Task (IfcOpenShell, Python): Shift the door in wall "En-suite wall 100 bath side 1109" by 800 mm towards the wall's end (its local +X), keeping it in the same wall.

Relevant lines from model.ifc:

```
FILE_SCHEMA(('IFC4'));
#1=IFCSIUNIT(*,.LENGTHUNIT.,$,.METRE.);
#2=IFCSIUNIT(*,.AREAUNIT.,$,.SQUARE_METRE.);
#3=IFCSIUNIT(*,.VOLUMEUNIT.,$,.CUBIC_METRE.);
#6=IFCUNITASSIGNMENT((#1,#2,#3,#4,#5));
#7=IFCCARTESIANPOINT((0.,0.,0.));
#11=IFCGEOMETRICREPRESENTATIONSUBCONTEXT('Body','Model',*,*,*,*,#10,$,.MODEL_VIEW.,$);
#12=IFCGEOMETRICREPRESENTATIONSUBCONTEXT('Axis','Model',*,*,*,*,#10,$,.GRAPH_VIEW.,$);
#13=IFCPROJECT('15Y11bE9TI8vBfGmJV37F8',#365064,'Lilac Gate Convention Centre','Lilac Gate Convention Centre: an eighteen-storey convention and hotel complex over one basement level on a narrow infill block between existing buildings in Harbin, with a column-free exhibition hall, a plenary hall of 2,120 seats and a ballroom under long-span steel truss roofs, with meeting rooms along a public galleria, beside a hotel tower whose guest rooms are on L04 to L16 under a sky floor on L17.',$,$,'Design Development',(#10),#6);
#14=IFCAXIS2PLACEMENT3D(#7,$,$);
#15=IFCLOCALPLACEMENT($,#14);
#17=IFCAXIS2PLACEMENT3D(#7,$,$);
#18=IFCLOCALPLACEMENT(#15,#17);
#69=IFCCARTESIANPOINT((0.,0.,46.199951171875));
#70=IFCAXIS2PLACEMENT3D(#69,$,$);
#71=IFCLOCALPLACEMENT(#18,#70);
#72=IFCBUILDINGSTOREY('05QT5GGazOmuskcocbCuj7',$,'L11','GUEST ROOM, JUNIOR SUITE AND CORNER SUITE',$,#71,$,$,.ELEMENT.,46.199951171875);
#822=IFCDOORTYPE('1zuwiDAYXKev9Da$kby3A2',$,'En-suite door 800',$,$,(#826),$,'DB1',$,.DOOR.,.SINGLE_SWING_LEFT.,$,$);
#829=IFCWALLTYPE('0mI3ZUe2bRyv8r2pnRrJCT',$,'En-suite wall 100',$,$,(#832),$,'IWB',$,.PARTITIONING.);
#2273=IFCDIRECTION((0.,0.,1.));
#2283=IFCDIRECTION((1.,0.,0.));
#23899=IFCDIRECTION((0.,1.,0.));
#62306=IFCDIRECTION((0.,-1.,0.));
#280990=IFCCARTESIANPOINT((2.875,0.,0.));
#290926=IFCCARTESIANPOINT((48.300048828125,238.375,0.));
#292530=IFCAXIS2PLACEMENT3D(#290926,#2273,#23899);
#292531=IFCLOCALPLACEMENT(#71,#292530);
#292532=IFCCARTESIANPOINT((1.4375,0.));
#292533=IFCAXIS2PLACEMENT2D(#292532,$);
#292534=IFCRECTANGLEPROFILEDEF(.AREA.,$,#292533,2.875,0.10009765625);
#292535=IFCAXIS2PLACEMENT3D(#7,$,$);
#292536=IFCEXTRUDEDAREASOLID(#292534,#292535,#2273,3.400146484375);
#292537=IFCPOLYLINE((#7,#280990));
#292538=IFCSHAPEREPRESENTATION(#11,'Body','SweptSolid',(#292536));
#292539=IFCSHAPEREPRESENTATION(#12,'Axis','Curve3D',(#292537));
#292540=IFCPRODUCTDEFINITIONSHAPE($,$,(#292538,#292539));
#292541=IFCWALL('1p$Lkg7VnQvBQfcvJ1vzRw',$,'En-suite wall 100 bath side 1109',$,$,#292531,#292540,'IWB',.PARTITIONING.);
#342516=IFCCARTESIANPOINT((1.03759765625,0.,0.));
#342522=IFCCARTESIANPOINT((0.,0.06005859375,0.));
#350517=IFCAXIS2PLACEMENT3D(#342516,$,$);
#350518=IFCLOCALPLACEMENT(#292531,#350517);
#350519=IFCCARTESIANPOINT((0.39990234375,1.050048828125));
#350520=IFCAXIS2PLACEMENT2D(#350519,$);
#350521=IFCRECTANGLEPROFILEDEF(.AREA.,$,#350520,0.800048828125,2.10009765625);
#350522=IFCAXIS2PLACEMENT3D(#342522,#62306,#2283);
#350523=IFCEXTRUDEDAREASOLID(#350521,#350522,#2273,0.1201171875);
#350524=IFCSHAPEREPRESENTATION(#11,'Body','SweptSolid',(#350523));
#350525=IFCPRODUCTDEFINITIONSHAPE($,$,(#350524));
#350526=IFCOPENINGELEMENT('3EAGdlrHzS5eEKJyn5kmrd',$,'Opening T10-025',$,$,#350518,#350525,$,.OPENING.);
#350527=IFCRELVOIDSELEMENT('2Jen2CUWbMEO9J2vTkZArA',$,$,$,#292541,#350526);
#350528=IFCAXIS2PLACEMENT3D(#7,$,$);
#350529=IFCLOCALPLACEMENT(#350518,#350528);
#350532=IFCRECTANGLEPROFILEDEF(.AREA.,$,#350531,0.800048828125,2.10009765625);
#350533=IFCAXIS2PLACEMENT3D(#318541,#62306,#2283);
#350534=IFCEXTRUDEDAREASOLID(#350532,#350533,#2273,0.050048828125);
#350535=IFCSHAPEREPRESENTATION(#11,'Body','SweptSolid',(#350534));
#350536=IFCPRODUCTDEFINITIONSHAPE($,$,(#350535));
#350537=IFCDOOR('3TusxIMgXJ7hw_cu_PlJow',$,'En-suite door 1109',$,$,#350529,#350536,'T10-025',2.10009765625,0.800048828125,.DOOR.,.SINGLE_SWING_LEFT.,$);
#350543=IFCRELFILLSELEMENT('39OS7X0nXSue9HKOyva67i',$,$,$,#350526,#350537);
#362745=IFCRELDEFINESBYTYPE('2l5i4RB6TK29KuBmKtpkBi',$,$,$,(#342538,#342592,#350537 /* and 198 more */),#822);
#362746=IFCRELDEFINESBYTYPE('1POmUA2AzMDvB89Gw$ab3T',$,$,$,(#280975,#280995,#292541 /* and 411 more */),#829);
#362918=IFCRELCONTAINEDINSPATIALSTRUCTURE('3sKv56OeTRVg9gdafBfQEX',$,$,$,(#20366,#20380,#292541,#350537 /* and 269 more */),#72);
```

```python
import ifcopenshell
import ifcopenshell.api.geometry
import ifcopenshell.util.placement
import ifcopenshell.util.unit

model = ifcopenshell.open("model.ifc")
unit_scale = ifcopenshell.util.unit.calculate_unit_scale(model)

door = model.by_id(350537)
opening = door.FillsVoids[0].RelatingOpeningElement
wall = opening.VoidsElements[0].RelatingBuildingElement

wall_matrix = ifcopenshell.util.placement.get_local_placement(wall.ObjectPlacement)
shift = wall_matrix[:3, 0] * 0.8 / unit_scale
before = ifcopenshell.util.placement.get_local_placement(door.ObjectPlacement)[:3, 3].copy()

# The door is placed relative to its opening, so it follows when the opening moves.
matrix = ifcopenshell.util.placement.get_local_placement(opening.ObjectPlacement)
matrix[:3, 3] += shift
ifcopenshell.api.geometry.edit_object_placement(
    model, product=opening, matrix=matrix, is_si=False, should_transform_children=True
)

after = ifcopenshell.util.placement.get_local_placement(door.ObjectPlacement)[:3, 3]
print("door moved by", (after - before).round(3) + 0.0)

model.write("model_updated.ifc")
```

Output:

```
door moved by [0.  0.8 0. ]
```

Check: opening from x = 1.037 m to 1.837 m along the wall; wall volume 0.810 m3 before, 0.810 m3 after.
